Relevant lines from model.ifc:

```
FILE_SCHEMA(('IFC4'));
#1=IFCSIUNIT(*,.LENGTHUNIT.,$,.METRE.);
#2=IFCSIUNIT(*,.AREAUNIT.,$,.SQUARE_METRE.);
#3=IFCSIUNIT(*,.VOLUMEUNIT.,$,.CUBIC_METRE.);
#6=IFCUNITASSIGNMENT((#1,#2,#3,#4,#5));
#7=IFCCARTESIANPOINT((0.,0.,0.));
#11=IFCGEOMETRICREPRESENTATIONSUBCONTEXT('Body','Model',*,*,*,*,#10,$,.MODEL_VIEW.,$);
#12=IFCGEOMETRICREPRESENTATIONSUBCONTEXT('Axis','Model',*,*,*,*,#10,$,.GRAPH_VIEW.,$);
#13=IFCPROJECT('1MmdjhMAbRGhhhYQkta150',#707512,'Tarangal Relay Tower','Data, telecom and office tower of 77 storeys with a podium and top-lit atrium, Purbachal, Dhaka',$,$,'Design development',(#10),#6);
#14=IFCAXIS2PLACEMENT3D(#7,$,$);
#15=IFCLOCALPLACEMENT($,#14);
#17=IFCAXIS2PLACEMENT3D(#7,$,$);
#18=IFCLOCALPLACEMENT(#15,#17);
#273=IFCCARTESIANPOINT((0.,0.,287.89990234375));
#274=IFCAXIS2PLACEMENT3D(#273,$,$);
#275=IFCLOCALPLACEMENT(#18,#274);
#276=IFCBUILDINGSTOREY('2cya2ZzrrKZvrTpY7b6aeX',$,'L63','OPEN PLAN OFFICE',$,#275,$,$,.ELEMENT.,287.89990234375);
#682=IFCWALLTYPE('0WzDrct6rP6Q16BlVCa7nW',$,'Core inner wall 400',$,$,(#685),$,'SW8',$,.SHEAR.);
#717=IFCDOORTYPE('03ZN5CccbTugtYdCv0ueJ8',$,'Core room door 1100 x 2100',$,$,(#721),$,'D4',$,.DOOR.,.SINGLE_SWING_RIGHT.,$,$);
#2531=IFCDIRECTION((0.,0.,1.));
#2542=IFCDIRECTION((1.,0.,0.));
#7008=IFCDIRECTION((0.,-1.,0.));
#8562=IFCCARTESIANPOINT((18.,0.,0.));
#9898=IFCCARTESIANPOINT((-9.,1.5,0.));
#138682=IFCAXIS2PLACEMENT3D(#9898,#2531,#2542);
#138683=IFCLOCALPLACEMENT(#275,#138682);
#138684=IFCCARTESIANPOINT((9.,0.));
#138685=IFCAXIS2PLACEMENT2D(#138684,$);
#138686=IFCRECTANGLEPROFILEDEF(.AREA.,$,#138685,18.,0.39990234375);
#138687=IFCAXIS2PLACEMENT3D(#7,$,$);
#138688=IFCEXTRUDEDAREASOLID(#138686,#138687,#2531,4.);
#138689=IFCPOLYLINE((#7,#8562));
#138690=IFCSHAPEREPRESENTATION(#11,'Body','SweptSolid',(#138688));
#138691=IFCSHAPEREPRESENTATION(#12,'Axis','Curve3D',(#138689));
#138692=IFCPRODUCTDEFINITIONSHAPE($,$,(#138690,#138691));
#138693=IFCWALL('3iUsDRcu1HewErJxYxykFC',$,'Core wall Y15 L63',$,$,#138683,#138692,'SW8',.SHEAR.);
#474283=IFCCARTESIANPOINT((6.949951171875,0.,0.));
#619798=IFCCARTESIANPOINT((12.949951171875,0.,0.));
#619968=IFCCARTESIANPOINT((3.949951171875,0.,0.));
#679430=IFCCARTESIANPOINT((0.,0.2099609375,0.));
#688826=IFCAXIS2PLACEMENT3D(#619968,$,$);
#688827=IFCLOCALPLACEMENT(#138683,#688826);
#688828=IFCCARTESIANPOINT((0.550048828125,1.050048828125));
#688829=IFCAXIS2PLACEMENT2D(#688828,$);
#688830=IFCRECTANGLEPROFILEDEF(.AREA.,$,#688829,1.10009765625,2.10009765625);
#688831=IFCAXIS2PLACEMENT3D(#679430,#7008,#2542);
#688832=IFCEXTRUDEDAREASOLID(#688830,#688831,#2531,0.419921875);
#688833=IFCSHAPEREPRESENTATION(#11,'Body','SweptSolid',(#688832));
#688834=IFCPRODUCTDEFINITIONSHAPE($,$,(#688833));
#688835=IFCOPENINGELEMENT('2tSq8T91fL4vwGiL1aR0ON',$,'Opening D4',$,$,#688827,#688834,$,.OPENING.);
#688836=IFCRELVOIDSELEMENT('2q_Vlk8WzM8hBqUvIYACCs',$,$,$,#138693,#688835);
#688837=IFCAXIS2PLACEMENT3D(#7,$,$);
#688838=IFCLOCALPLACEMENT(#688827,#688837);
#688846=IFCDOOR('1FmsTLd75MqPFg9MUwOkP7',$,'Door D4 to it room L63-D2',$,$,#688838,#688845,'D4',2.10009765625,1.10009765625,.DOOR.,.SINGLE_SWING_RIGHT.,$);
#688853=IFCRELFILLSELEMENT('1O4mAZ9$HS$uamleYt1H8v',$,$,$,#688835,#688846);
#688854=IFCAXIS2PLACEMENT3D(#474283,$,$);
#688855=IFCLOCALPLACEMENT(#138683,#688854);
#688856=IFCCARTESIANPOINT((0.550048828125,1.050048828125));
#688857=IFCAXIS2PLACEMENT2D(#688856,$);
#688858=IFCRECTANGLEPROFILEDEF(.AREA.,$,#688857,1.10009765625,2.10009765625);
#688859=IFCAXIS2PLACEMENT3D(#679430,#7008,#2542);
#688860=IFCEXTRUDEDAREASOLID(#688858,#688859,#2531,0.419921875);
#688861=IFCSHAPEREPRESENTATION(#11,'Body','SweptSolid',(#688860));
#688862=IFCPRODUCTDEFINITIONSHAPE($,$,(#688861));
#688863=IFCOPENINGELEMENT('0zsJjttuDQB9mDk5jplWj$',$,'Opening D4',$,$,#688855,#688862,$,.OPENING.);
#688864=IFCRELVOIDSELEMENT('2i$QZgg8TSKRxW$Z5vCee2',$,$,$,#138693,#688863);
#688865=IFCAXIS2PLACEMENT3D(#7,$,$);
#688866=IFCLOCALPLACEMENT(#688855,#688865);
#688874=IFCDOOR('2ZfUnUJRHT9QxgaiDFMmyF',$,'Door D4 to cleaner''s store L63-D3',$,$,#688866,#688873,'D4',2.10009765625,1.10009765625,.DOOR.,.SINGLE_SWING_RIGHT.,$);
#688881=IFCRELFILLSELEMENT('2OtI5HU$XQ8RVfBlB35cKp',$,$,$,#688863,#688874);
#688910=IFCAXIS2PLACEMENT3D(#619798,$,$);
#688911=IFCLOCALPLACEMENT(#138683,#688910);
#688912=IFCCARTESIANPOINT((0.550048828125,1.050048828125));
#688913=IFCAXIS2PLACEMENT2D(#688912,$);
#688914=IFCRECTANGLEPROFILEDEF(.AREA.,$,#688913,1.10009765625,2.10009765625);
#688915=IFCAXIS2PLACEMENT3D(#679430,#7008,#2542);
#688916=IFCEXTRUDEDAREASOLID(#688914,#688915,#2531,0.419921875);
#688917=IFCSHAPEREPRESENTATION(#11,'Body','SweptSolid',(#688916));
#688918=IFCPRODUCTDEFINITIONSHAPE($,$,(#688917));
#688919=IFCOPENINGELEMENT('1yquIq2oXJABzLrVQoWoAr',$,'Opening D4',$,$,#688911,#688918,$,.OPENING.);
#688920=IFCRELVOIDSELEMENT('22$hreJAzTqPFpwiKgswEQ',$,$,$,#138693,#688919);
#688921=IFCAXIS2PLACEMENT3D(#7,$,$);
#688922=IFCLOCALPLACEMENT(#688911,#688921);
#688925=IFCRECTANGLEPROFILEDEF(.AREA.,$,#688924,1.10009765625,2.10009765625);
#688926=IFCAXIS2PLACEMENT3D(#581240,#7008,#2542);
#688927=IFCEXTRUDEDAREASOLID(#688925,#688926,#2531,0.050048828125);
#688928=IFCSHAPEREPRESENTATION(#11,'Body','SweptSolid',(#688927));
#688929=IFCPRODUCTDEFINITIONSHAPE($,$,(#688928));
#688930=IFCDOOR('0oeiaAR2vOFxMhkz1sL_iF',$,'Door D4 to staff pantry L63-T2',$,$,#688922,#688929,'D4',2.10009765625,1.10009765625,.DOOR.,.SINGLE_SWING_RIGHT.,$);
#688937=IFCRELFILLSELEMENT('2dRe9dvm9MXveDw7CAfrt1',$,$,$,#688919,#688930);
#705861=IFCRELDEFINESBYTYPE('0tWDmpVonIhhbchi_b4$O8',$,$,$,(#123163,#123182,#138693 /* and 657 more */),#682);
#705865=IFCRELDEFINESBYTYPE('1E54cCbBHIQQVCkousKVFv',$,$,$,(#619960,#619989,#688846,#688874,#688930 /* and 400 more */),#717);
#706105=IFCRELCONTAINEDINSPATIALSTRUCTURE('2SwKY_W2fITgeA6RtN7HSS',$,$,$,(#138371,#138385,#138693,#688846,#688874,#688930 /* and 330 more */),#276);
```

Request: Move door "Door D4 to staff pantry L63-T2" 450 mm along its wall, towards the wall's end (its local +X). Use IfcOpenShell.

```python
import ifcopenshell
import ifcopenshell.api.geometry
import ifcopenshell.util.placement

model = ifcopenshell.open("model.ifc")

door = model.by_guid("0oeiaAR2vOFxMhkz1sL_iF")
opening = door.FillsVoids[0].RelatingOpeningElement
wall = opening.VoidsElements[0].RelatingBuildingElement

wall_matrix = ifcopenshell.util.placement.get_local_placement(wall.ObjectPlacement)
shift = wall_matrix[:3, 0] * 0.45
before = ifcopenshell.util.placement.get_local_placement(door.ObjectPlacement)[:3, 3].copy()

# The door is placed relative to its opening, so it follows when the opening moves.
matrix = ifcopenshell.util.placement.get_local_placement(opening.ObjectPlacement)
matrix[:3, 3] += shift
ifcopenshell.api.geometry.edit_object_placement(
    model, product=opening, matrix=matrix, is_si=False, should_transform_children=True
)

after = ifcopenshell.util.placement.get_local_placement(door.ObjectPlacement)[:3, 3]
print("door moved by", (after - before).round(3) + 0.0)

model.write("model-out.ifc")
```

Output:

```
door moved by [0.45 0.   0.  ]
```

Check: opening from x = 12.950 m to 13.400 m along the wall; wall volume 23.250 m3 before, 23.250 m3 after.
